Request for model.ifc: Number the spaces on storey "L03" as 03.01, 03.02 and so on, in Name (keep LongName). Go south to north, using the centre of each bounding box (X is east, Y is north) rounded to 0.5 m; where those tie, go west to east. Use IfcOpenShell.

First a look at what the model holds.

```python
import ifcopenshell
import ifcopenshell.util.element
import ifcopenshell.util.placement

model = ifcopenshell.open("model.ifc")
print(model.schema)
storey = next(s for s in model.by_type("IfcBuildingStorey") if s.Name == "L03")
spaces = [e for e in ifcopenshell.util.element.get_decomposition(storey) if e.is_a("IfcSpace")]
for e in sorted(spaces, key=lambda e: e.id()):
    origin = ifcopenshell.util.placement.get_local_placement(e.ObjectPlacement)[:3, 3]
    print(e.id(), e.Name, e.LongName, origin.round(2) + 0.0, sep=" | ")
```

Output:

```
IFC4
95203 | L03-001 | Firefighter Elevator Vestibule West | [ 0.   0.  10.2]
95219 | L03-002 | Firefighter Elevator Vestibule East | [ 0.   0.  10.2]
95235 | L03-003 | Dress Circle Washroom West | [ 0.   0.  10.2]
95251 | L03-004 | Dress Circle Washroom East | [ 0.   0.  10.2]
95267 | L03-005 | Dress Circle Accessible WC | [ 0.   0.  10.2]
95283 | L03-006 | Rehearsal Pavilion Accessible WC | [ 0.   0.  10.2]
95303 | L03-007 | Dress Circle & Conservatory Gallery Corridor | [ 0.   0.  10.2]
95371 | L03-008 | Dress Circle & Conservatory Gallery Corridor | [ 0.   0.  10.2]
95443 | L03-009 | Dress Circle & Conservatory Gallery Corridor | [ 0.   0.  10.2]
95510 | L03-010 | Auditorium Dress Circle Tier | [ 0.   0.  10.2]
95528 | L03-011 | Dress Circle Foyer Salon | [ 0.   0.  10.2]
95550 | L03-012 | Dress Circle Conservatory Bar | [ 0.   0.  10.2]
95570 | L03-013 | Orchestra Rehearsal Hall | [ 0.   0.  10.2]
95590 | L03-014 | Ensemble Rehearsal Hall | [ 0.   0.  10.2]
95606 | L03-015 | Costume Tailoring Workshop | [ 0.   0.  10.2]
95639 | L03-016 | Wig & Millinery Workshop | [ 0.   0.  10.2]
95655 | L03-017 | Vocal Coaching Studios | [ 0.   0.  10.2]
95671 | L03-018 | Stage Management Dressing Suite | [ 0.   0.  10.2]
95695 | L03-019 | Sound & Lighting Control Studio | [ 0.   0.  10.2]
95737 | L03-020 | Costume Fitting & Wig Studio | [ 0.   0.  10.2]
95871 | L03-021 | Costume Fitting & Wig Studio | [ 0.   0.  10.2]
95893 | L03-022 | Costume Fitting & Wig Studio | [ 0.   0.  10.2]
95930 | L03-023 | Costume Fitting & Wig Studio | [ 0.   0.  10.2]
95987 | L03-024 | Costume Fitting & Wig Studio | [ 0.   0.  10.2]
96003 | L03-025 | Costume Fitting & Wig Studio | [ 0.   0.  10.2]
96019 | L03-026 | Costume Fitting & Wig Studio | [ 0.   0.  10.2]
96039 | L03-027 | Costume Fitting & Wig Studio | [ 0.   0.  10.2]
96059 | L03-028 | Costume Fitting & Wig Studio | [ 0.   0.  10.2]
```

```python
import ifcopenshell
import ifcopenshell.geom
import ifcopenshell.util.element
import ifcopenshell.util.shape

model = ifcopenshell.open("model.ifc")
settings = ifcopenshell.geom.settings()
settings.set("use-world-coords", True)


def centre(element):
    shape = ifcopenshell.geom.create_shape(settings, element)
    return ifcopenshell.util.shape.get_bbox_centroid(shape.geometry)


storey = next(s for s in model.by_type("IfcBuildingStorey") if s.Name == "L03")
spaces = [e for e in ifcopenshell.util.element.get_decomposition(storey) if e.is_a("IfcSpace")]

# Insertion points can sit at a corner or the storey origin, so sort by the geometry (in metres).
centres = {e: centre(e) for e in spaces}
spaces.sort(key=lambda e: (round(centres[e][1] / 0.5), centres[e][0]))

for i, e in enumerate(spaces, start=1):
    number = f"03.{i:02d}"
    e.Name = number
    print(e.id(), number)

model.write("model-out.ifc")
```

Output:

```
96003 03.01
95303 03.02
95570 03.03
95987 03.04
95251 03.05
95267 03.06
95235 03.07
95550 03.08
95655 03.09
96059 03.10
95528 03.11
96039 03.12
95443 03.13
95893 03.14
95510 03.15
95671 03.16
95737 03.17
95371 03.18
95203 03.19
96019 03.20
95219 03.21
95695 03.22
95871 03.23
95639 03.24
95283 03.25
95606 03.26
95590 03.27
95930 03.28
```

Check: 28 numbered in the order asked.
